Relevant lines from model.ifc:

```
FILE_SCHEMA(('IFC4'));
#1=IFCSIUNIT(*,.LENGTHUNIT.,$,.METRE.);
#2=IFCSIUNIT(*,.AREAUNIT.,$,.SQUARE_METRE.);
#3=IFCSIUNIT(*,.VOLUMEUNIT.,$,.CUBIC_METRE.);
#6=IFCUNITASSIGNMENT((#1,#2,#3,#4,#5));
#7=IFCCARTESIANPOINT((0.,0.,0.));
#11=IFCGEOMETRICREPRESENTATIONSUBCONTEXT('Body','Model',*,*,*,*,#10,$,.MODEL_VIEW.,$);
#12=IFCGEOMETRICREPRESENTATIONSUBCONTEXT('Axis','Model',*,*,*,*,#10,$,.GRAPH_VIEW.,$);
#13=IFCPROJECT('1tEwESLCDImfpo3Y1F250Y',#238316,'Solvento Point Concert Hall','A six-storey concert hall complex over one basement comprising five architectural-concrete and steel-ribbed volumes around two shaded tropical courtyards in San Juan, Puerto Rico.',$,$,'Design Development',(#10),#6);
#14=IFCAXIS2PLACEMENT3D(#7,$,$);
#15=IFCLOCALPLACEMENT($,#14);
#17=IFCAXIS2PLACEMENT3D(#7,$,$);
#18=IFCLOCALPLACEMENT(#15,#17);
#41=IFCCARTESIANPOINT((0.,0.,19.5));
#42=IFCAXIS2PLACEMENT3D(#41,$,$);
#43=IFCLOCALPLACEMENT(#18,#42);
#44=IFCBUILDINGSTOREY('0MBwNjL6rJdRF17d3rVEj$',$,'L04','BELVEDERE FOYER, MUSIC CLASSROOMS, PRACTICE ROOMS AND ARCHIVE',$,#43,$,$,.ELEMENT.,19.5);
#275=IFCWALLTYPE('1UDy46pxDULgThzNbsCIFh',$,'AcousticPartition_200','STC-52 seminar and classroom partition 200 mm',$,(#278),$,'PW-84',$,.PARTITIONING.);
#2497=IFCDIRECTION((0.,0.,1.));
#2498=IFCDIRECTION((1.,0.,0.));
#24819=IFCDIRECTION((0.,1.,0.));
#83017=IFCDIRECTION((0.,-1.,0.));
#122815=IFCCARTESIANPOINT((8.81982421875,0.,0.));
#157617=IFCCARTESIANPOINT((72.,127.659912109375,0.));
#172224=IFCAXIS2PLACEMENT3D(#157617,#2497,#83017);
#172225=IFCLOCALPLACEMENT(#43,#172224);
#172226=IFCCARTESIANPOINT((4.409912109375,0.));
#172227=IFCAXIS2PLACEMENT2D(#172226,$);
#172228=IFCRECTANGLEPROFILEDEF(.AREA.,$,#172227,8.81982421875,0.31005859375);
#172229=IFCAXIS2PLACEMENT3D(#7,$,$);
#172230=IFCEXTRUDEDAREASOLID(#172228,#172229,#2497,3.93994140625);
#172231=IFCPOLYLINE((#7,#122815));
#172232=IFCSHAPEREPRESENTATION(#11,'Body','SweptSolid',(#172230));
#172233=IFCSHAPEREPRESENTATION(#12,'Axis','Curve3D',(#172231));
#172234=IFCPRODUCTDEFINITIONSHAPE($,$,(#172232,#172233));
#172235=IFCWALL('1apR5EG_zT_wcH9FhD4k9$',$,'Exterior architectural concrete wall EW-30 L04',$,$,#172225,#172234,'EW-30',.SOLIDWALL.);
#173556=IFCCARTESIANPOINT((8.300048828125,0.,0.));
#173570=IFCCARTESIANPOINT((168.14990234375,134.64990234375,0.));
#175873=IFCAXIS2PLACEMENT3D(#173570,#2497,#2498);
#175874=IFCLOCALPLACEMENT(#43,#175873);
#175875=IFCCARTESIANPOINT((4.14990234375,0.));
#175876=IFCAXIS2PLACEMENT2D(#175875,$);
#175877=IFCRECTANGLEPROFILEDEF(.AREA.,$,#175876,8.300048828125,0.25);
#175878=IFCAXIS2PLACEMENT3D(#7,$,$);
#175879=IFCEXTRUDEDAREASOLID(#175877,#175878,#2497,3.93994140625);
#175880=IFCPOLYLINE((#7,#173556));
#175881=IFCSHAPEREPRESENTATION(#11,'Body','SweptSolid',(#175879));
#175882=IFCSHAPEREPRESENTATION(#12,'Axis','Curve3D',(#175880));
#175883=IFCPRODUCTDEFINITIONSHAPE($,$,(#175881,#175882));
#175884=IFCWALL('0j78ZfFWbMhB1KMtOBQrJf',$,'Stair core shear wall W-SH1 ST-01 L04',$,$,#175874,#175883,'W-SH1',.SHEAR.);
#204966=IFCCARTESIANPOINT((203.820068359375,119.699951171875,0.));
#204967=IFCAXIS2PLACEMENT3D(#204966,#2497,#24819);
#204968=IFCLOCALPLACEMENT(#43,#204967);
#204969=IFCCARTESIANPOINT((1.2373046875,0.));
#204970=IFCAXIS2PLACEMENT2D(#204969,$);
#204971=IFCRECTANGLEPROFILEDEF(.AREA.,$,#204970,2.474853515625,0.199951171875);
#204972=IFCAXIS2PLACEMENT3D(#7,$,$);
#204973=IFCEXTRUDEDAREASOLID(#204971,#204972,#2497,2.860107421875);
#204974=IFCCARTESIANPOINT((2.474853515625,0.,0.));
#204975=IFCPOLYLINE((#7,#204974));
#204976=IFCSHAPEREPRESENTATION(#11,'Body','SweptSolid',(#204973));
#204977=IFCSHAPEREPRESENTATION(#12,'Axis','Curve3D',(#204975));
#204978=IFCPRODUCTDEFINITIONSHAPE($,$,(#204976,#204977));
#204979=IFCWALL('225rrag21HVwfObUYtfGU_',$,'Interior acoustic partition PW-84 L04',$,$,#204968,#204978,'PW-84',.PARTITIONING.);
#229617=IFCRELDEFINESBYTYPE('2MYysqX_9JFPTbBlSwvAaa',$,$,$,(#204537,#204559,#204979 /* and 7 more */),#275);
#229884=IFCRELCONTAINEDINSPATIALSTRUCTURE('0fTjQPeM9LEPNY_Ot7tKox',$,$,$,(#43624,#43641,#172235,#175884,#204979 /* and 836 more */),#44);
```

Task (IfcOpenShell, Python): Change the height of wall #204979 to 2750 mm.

```python
import ifcopenshell
import ifcopenshell.geom
import ifcopenshell.util.representation
import ifcopenshell.util.shape

model = ifcopenshell.open("model.ifc")
settings = ifcopenshell.geom.settings()


def volume(element):
    """Net volume in cubic metres, openings subtracted."""
    shape = ifcopenshell.geom.create_shape(settings, element)
    return ifcopenshell.util.shape.get_volume(shape.geometry)


wall = model.by_guid("225rrag21HVwfObUYtfGU_")
before = volume(wall)

body = ifcopenshell.util.representation.get_representation(wall, "Model", "Body")
solid = body.Items[0]
old_height = solid.Depth
solid.Depth = 2.75
after = volume(wall)

print(f"height {old_height:g} -> {solid.Depth:g}, volume {before:.3f} -> {after:.3f} m3")

model.write("model_updated.ifc")
```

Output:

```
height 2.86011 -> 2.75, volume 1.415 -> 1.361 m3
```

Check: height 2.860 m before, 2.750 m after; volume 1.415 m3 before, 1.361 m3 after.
